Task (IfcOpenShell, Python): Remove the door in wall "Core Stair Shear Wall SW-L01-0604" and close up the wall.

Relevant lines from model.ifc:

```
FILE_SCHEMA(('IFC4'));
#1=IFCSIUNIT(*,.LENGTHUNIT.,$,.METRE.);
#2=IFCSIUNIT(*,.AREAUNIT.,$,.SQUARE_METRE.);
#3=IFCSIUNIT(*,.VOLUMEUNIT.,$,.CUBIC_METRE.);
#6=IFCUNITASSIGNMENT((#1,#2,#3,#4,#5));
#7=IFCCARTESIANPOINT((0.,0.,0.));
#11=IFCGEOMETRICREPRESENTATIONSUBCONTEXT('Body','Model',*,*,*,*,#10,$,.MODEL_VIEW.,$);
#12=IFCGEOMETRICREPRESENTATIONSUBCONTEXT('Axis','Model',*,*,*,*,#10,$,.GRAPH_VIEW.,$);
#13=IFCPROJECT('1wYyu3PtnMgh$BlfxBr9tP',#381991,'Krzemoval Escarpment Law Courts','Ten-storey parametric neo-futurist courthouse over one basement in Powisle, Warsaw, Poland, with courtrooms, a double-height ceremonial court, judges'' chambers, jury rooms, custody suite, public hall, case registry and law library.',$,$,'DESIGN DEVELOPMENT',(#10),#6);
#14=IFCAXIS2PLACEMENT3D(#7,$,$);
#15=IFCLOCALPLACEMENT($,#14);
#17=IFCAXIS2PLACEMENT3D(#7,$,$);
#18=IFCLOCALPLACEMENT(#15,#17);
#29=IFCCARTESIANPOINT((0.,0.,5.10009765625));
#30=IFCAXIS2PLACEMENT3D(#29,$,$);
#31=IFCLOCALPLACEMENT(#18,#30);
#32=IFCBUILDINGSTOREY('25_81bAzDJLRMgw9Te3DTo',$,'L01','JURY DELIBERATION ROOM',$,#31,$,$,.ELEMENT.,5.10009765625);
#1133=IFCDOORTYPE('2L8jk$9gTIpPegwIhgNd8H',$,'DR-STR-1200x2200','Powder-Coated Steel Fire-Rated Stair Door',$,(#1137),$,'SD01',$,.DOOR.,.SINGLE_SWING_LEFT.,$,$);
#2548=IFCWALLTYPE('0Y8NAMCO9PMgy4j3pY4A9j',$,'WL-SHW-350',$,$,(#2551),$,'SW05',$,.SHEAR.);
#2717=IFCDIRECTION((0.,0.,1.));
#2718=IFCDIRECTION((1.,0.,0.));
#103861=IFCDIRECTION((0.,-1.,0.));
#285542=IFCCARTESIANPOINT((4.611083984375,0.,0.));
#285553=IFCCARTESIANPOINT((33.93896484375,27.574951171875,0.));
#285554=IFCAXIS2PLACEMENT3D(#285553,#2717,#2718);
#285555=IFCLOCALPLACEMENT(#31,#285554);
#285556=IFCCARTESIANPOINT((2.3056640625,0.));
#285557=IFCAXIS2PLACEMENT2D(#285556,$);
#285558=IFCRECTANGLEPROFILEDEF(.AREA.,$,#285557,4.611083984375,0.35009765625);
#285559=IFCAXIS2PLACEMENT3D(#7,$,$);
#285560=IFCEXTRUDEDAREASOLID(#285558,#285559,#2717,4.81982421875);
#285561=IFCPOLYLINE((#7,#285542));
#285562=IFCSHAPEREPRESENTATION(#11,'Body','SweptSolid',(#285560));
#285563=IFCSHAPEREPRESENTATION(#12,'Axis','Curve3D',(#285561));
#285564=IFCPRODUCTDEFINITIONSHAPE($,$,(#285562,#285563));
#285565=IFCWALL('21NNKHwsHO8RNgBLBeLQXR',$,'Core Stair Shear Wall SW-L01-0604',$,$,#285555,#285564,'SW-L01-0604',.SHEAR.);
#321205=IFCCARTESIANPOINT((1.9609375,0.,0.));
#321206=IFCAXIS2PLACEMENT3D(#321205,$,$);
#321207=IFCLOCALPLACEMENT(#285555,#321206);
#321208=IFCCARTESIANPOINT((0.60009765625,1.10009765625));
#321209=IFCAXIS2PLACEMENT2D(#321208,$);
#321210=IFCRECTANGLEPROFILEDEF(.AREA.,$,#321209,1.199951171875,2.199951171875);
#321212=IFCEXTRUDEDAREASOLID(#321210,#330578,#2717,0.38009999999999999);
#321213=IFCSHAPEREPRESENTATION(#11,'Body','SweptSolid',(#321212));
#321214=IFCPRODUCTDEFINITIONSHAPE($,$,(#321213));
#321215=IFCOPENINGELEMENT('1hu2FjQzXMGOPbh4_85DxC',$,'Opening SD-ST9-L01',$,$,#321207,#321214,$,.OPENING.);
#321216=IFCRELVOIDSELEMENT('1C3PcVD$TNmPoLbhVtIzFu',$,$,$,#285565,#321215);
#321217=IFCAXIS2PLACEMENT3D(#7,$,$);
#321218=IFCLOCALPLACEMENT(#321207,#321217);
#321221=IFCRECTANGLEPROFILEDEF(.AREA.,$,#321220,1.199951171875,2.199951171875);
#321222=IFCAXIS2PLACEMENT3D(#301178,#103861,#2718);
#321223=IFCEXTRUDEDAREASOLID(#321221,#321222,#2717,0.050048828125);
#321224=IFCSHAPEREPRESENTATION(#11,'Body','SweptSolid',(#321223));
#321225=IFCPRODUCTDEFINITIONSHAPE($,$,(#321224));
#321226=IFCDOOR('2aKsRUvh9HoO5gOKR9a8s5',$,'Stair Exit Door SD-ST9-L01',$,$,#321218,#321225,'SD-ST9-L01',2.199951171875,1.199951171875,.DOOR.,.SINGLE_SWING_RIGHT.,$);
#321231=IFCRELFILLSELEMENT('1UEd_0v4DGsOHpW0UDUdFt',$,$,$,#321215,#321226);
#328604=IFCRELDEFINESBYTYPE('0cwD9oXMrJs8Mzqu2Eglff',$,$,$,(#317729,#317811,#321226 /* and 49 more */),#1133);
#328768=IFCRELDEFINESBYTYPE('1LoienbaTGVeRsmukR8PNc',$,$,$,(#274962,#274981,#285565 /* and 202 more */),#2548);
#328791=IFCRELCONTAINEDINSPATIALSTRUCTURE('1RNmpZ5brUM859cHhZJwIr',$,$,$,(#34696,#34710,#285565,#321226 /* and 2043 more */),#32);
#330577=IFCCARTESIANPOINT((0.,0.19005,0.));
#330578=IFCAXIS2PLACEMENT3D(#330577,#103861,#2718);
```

```python
import ifcopenshell
import ifcopenshell.api.feature
import ifcopenshell.api.root
import ifcopenshell.geom
import ifcopenshell.util.shape

model = ifcopenshell.open("model.ifc")
settings = ifcopenshell.geom.settings()


def volume(element):
    """Net volume in cubic metres, openings subtracted."""
    shape = ifcopenshell.geom.create_shape(settings, element)
    return ifcopenshell.util.shape.get_volume(shape.geometry)


door = model.by_guid("2aKsRUvh9HoO5gOKR9a8s5")
opening = door.FillsVoids[0].RelatingOpeningElement
wall = opening.VoidsElements[0].RelatingBuildingElement
before = volume(wall)

ifcopenshell.api.root.remove_product(model, product=door)
ifcopenshell.api.feature.remove_feature(model, feature=opening)

after = volume(wall)

print(f"wall volume {before:.3f} -> {after:.3f} m3")

model.write("model-out.ifc")
```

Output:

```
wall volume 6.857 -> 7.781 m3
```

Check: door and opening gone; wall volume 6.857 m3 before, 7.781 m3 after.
